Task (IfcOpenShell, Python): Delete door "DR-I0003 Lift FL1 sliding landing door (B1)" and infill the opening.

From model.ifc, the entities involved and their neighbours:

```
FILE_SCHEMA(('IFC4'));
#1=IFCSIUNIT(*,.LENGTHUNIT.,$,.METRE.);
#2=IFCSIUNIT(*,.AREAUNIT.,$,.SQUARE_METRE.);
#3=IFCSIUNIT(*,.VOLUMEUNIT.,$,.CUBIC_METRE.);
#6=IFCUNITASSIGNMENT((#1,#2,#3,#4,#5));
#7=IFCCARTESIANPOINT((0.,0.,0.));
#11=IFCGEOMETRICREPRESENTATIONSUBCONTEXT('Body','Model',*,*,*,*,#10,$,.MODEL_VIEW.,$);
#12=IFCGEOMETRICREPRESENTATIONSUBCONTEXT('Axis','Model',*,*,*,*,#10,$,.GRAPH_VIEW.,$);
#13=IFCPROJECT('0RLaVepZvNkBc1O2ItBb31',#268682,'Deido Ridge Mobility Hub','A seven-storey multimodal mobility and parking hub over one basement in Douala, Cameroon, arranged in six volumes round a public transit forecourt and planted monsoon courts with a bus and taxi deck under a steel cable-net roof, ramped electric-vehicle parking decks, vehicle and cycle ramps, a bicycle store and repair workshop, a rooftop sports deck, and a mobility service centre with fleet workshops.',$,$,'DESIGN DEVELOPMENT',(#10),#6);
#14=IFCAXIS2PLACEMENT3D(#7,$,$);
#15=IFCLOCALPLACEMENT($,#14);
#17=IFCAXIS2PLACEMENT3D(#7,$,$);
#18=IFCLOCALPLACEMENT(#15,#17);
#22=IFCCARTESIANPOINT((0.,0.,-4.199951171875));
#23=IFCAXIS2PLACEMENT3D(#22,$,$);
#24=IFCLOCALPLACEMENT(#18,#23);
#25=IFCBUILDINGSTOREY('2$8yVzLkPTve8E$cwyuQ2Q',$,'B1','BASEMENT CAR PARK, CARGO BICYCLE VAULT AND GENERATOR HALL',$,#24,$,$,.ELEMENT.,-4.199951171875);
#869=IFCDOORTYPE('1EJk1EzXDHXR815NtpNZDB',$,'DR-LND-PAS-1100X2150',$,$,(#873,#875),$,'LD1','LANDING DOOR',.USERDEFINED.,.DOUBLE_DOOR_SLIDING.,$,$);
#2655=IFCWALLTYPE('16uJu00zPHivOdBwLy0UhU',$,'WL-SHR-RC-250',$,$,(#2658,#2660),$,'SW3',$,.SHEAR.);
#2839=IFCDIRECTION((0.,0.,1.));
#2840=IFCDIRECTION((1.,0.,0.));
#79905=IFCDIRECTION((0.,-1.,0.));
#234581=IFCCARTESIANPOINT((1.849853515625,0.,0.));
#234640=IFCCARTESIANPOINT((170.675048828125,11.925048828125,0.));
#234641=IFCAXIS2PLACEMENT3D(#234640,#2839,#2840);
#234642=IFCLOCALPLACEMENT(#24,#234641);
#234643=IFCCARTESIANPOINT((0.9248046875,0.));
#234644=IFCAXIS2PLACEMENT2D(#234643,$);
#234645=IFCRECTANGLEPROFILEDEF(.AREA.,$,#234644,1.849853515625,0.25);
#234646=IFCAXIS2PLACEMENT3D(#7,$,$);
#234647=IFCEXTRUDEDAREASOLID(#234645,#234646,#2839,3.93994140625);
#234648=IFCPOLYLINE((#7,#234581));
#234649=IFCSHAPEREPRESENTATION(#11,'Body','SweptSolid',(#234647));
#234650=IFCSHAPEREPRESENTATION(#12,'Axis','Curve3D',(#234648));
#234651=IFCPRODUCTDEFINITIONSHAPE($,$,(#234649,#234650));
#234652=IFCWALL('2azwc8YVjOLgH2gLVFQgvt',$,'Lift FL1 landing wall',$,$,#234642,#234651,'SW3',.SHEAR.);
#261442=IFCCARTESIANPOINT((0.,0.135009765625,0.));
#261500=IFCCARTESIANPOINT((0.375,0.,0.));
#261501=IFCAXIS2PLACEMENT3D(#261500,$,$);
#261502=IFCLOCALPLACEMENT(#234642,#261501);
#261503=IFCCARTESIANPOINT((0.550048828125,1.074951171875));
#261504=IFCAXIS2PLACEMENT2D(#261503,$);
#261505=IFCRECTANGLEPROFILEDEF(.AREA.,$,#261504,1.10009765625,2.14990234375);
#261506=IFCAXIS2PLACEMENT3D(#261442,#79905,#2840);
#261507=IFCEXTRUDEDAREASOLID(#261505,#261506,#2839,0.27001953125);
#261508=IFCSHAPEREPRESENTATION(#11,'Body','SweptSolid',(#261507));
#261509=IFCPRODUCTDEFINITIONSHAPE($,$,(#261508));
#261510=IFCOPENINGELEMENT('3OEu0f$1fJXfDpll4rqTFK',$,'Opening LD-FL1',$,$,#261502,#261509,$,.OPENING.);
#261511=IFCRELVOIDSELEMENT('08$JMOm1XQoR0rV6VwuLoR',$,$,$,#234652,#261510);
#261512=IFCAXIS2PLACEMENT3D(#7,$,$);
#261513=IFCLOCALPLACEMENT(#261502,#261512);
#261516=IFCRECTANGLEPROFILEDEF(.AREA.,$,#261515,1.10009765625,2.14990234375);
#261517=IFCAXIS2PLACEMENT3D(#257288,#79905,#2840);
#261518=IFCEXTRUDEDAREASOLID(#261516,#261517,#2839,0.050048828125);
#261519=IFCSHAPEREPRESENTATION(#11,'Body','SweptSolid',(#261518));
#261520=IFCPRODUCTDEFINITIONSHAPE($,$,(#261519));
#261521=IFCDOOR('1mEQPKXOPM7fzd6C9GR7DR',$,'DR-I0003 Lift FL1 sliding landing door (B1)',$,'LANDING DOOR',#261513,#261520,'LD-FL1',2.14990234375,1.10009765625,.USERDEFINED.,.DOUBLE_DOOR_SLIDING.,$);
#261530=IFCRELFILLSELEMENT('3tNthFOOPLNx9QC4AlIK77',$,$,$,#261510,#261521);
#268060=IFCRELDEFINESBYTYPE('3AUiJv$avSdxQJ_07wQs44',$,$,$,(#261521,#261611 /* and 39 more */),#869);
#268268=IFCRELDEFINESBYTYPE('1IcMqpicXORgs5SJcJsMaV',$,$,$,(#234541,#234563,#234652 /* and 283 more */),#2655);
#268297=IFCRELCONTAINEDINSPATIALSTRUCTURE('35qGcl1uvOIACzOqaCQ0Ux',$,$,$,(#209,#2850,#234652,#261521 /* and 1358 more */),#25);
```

```python
import ifcopenshell
import ifcopenshell.api.feature
import ifcopenshell.api.root
import ifcopenshell.geom
import ifcopenshell.util.shape

model = ifcopenshell.open("model.ifc")
settings = ifcopenshell.geom.settings()


def volume(element):
    """Net volume in cubic metres, openings subtracted."""
    shape = ifcopenshell.geom.create_shape(settings, element)
    return ifcopenshell.util.shape.get_volume(shape.geometry)


door = model.by_id(261521)
opening = door.FillsVoids[0].RelatingOpeningElement
wall = opening.VoidsElements[0].RelatingBuildingElement
before = volume(wall)

ifcopenshell.api.root.remove_product(model, product=door)
ifcopenshell.api.feature.remove_feature(model, feature=opening)

after = volume(wall)

print(f"wall volume {before:.3f} -> {after:.3f} m3")

model.write("model_v2.ifc")
```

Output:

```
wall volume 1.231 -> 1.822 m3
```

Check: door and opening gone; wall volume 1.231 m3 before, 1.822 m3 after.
